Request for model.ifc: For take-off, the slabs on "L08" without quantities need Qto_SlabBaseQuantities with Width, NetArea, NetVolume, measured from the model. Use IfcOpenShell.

First a look at what the model holds.

```python
import ifcopenshell
import ifcopenshell.util.element
import ifcopenshell.util.unit

model = ifcopenshell.open("model.ifc")
print(model.schema)
for unit_type in ("LENGTHUNIT", "AREAUNIT", "VOLUMEUNIT"):
    print(unit_type, ifcopenshell.util.unit.calculate_unit_scale(model, unit_type))
storey = next(s for s in model.by_type("IfcBuildingStorey") if s.Name == "L08")
slabs = [e for e in ifcopenshell.util.element.get_decomposition(storey) if e.is_a("IfcSlab")]
for e in sorted(slabs, key=lambda e: e.id()):
    print(e.id(), e.is_a(), e.Name, list(ifcopenshell.util.element.get_psets(e, qtos_only=True)), sep=" | ")
```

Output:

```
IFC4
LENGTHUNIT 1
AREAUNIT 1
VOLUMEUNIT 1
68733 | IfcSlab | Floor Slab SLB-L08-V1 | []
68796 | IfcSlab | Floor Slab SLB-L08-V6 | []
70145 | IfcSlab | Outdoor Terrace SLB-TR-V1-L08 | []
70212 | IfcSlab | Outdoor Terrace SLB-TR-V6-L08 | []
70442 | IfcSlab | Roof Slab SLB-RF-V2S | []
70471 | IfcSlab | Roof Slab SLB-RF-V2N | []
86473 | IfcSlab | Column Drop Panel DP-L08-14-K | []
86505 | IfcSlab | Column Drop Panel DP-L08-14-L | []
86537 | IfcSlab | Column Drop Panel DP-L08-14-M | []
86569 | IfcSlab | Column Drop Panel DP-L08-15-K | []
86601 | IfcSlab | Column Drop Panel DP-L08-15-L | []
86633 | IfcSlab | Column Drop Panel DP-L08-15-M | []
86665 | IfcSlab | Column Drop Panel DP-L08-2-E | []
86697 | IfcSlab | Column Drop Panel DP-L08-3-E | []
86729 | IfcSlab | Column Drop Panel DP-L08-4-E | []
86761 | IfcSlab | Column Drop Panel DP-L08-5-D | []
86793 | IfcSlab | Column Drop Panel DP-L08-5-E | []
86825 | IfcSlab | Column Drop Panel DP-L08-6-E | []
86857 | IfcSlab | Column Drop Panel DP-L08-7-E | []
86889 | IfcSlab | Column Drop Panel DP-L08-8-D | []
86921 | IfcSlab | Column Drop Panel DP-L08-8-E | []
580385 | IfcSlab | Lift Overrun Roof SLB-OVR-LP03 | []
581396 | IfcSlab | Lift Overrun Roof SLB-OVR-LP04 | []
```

```python
import ifcopenshell
import ifcopenshell.api.pset
import ifcopenshell.geom
import ifcopenshell.util.element
import ifcopenshell.util.shape
import ifcopenshell.util.unit

model = ifcopenshell.open("model.ifc")
unit_scale = ifcopenshell.util.unit.calculate_unit_scale(model)
area_scale = ifcopenshell.util.unit.calculate_unit_scale(model, "AREAUNIT")
volume_scale = ifcopenshell.util.unit.calculate_unit_scale(model, "VOLUMEUNIT")
settings = ifcopenshell.geom.settings()

storey = next(s for s in model.by_type("IfcBuildingStorey") if s.Name == "L08")
slabs = [e for e in ifcopenshell.util.element.get_decomposition(storey) if e.is_a("IfcSlab")]

for e in sorted(slabs, key=lambda e: e.id()):
    if ifcopenshell.util.element.get_psets(e, qtos_only=True, should_inherit=False):
        continue
    # Geometry comes back in metres, in the element's own axes.
    shape = ifcopenshell.geom.create_shape(settings, e)
    values = {
        "Width": ifcopenshell.util.shape.get_z(shape.geometry) / unit_scale,
        "NetArea": ifcopenshell.util.shape.get_footprint_area(shape.geometry) / area_scale,
        "NetVolume": ifcopenshell.util.shape.get_volume(shape.geometry) / volume_scale,
    }
    qto = ifcopenshell.api.pset.add_qto(model, product=e, name="Qto_SlabBaseQuantities")
    ifcopenshell.api.pset.edit_qto(model, qto=qto, properties=values)
    print(e.id(), {k: round(v, 3) for k, v in values.items()})

model.write("model_v2.ifc")
```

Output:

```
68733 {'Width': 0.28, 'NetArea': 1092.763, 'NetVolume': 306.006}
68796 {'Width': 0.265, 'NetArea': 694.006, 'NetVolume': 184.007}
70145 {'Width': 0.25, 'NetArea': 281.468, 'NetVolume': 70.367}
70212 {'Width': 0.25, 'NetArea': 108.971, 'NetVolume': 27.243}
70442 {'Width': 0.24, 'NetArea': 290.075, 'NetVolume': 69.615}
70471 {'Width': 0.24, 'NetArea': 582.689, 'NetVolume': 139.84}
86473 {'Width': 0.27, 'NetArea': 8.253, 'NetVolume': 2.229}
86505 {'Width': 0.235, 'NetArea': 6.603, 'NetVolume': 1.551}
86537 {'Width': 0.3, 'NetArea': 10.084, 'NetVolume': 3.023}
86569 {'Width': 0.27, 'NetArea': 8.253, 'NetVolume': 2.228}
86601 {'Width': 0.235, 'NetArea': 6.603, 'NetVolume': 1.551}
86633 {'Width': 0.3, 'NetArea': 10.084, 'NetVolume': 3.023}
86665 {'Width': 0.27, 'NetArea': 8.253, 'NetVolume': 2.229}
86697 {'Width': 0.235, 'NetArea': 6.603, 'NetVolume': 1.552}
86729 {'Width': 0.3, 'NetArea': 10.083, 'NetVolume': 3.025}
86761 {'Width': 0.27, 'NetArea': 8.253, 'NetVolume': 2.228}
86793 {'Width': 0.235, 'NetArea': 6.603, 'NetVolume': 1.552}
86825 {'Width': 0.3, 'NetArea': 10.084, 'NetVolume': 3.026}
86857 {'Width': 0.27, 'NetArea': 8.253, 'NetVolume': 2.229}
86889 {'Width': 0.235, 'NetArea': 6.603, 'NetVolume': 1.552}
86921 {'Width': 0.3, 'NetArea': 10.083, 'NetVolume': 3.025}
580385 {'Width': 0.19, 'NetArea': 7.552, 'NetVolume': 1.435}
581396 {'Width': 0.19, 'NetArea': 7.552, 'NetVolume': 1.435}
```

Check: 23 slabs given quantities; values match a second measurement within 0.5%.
